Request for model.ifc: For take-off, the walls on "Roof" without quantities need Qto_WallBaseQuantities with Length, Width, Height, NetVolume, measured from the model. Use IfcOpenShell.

First a look at what the model holds.

```python
import ifcopenshell
import ifcopenshell.util.element
import ifcopenshell.util.unit

model = ifcopenshell.open("model.ifc")
print(model.schema)
for unit_type in ("LENGTHUNIT", "AREAUNIT", "VOLUMEUNIT"):
    print(unit_type, ifcopenshell.util.unit.calculate_unit_scale(model, unit_type))
storey = next(s for s in model.by_type("IfcBuildingStorey") if s.Name == "Roof")
walls = [e for e in ifcopenshell.util.element.get_decomposition(storey) if e.is_a("IfcWall")]
for e in sorted(walls, key=lambda e: e.id()):
    print(e.id(), e.is_a(), e.Name, list(ifcopenshell.util.element.get_psets(e, qtos_only=True)), sep=" | ")
```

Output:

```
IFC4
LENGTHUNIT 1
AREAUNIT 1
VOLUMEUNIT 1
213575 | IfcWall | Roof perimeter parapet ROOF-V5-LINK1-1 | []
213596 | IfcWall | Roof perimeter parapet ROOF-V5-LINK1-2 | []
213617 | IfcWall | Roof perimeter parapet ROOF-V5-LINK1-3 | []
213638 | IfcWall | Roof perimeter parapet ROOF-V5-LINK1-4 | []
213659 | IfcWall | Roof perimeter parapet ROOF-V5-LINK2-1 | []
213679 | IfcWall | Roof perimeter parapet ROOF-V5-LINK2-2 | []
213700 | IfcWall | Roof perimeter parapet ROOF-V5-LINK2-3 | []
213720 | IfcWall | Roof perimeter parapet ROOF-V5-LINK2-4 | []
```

```python
import ifcopenshell
import ifcopenshell.api.pset
import ifcopenshell.geom
import ifcopenshell.util.element
import ifcopenshell.util.shape
import ifcopenshell.util.unit

model = ifcopenshell.open("model.ifc")
unit_scale = ifcopenshell.util.unit.calculate_unit_scale(model)
volume_scale = ifcopenshell.util.unit.calculate_unit_scale(model, "VOLUMEUNIT")
settings = ifcopenshell.geom.settings()

storey = next(s for s in model.by_type("IfcBuildingStorey") if s.Name == "Roof")
walls = [e for e in ifcopenshell.util.element.get_decomposition(storey) if e.is_a("IfcWall")]

for e in sorted(walls, key=lambda e: e.id()):
    if ifcopenshell.util.element.get_psets(e, qtos_only=True, should_inherit=False):
        continue
    # Geometry comes back in metres, in the element's own axes.
    shape = ifcopenshell.geom.create_shape(settings, e)
    values = {
        "Length": ifcopenshell.util.shape.get_x(shape.geometry) / unit_scale,
        "Width": ifcopenshell.util.shape.get_y(shape.geometry) / unit_scale,
        "Height": ifcopenshell.util.shape.get_z(shape.geometry) / unit_scale,
        "NetVolume": ifcopenshell.util.shape.get_volume(shape.geometry) / volume_scale,
    }
    qto = ifcopenshell.api.pset.add_qto(model, product=e, name="Qto_WallBaseQuantities")
    ifcopenshell.api.pset.edit_qto(model, qto=qto, properties=values)
    print(e.id(), {k: round(v, 3) for k, v in values.items()})

model.write("model-out.ifc")
```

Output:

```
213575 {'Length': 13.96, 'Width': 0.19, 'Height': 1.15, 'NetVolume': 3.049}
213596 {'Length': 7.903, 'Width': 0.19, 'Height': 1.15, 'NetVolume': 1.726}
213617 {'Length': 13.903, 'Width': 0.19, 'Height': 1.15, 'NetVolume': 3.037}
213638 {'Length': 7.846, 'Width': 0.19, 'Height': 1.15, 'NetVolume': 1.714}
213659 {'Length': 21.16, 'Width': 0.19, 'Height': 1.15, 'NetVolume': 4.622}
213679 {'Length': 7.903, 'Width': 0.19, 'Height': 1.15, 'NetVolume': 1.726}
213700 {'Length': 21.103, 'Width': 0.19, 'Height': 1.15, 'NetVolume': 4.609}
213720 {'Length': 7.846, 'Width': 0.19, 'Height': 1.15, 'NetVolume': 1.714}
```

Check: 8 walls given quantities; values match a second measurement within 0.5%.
